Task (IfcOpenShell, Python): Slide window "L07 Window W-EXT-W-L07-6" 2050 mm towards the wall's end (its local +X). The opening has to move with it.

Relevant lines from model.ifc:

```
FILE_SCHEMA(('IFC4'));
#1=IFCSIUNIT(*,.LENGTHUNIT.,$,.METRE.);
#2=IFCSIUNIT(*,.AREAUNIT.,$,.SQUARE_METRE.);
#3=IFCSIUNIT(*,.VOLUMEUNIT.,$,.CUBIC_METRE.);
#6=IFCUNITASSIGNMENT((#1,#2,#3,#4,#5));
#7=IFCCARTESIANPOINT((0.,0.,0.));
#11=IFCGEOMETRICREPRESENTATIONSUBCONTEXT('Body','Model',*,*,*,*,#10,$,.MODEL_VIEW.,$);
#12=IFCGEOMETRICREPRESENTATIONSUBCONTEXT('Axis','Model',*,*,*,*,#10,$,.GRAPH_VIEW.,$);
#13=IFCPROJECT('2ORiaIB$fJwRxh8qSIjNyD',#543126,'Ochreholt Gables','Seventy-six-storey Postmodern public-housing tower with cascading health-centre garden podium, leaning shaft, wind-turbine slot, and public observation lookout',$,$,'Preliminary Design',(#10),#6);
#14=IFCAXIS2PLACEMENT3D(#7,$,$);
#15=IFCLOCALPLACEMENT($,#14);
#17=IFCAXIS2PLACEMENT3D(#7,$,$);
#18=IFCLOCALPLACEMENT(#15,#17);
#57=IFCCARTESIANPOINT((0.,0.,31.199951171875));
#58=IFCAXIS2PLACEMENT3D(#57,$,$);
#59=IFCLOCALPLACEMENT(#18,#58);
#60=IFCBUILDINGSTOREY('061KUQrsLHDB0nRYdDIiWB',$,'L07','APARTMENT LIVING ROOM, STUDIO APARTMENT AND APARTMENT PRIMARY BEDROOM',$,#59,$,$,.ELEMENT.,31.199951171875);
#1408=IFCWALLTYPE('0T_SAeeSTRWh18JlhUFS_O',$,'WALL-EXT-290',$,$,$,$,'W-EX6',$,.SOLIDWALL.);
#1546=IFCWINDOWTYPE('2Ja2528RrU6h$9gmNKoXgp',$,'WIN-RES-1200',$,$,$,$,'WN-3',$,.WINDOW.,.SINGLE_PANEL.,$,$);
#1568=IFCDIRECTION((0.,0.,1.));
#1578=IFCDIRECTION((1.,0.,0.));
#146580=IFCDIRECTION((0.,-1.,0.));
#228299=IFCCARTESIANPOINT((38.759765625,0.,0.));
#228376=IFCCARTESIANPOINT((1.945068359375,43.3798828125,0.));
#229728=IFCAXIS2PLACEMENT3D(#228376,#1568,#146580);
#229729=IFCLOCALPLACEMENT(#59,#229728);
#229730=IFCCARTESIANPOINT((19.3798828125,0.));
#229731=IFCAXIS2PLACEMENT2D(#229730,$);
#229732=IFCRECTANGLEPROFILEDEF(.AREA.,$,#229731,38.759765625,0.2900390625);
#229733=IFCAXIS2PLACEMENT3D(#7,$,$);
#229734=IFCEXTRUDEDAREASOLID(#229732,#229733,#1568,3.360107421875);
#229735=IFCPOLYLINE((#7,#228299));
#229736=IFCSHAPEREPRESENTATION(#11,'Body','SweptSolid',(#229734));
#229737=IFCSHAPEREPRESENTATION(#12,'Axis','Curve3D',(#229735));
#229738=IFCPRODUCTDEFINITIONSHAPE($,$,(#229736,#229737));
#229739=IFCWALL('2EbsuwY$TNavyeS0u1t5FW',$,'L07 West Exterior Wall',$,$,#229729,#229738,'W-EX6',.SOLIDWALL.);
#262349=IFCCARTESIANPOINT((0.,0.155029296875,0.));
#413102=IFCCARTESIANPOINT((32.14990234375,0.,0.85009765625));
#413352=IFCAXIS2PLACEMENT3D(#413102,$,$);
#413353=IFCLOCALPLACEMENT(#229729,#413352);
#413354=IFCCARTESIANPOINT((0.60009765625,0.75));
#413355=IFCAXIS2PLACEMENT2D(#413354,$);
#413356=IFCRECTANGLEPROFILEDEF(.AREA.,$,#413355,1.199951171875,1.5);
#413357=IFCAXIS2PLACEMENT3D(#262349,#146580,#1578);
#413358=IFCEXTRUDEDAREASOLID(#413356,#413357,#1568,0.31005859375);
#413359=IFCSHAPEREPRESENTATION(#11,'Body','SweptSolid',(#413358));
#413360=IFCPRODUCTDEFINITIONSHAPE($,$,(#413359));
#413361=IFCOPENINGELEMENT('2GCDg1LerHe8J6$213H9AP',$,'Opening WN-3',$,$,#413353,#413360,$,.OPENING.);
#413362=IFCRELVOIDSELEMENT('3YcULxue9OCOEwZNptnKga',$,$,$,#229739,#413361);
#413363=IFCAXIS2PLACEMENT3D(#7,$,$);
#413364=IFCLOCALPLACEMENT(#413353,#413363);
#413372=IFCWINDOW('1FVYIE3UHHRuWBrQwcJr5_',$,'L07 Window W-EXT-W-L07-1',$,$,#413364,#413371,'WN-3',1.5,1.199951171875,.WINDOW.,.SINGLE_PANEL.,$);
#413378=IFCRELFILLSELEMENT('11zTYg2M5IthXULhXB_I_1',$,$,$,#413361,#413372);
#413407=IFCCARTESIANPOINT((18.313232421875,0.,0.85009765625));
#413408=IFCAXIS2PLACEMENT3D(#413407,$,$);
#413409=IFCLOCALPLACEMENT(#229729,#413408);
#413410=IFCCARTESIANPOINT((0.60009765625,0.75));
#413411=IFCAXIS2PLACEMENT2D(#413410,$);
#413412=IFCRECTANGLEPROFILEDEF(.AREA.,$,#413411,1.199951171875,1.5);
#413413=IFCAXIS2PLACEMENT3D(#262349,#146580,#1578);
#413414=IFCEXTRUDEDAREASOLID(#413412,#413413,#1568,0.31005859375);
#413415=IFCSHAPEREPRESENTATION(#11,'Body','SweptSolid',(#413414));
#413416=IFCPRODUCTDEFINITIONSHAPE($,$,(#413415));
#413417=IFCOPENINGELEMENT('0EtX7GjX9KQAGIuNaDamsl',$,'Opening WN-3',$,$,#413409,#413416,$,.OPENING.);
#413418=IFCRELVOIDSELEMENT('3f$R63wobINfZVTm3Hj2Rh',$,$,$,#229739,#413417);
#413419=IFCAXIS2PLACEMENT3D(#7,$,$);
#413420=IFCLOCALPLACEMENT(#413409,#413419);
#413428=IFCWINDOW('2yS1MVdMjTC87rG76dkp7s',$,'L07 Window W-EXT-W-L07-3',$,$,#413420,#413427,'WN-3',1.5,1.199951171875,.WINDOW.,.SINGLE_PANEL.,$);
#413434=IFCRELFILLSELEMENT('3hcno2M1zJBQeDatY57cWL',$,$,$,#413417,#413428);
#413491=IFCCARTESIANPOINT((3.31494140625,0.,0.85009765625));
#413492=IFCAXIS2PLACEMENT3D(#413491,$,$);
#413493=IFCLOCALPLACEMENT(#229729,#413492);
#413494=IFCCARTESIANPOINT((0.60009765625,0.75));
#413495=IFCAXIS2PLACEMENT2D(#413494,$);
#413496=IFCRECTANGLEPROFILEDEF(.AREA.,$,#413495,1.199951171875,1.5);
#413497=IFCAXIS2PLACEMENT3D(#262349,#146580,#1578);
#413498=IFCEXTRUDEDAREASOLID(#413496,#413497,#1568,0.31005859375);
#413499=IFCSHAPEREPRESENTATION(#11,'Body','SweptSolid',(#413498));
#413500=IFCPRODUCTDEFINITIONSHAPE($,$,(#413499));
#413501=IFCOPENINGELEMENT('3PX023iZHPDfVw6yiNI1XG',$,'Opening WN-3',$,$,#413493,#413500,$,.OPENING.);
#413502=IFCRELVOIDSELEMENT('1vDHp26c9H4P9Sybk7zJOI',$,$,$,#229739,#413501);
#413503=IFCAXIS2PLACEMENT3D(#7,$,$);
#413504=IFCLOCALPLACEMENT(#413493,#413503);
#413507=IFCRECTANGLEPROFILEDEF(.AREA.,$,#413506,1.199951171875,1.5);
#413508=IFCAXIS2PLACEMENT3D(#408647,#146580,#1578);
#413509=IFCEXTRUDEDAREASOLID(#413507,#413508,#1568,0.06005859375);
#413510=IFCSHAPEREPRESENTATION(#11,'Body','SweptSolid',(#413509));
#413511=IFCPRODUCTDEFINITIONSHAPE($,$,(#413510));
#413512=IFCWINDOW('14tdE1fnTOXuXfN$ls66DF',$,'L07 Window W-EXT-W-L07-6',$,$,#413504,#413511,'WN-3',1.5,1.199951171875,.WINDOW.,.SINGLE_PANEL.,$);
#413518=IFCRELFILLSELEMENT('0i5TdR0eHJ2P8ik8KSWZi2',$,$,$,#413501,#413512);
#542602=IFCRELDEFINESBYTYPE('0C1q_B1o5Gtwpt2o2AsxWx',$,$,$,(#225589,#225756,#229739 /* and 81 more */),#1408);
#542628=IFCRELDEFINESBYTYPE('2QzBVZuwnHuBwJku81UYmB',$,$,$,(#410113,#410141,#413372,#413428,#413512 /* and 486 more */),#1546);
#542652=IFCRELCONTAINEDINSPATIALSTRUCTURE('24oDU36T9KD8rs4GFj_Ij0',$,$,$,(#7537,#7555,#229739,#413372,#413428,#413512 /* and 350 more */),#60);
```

```python
import ifcopenshell
import ifcopenshell.api.geometry
import ifcopenshell.util.placement

model = ifcopenshell.open("model.ifc")

window = model.by_guid("14tdE1fnTOXuXfN$ls66DF")
opening = window.FillsVoids[0].RelatingOpeningElement
wall = opening.VoidsElements[0].RelatingBuildingElement

wall_matrix = ifcopenshell.util.placement.get_local_placement(wall.ObjectPlacement)
shift = wall_matrix[:3, 0] * 2.05
before = ifcopenshell.util.placement.get_local_placement(window.ObjectPlacement)[:3, 3].copy()

# The window is placed relative to its opening, so it follows when the opening moves.
matrix = ifcopenshell.util.placement.get_local_placement(opening.ObjectPlacement)
matrix[:3, 3] += shift
ifcopenshell.api.geometry.edit_object_placement(
    model, product=opening, matrix=matrix, is_si=False, should_transform_children=True
)

after = ifcopenshell.util.placement.get_local_placement(window.ObjectPlacement)[:3, 3]
print("window moved by", (after - before).round(3) + 0.0)

model.write("model_edited.ifc")
```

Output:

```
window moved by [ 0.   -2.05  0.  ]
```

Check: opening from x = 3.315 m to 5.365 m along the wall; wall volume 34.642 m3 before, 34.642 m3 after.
